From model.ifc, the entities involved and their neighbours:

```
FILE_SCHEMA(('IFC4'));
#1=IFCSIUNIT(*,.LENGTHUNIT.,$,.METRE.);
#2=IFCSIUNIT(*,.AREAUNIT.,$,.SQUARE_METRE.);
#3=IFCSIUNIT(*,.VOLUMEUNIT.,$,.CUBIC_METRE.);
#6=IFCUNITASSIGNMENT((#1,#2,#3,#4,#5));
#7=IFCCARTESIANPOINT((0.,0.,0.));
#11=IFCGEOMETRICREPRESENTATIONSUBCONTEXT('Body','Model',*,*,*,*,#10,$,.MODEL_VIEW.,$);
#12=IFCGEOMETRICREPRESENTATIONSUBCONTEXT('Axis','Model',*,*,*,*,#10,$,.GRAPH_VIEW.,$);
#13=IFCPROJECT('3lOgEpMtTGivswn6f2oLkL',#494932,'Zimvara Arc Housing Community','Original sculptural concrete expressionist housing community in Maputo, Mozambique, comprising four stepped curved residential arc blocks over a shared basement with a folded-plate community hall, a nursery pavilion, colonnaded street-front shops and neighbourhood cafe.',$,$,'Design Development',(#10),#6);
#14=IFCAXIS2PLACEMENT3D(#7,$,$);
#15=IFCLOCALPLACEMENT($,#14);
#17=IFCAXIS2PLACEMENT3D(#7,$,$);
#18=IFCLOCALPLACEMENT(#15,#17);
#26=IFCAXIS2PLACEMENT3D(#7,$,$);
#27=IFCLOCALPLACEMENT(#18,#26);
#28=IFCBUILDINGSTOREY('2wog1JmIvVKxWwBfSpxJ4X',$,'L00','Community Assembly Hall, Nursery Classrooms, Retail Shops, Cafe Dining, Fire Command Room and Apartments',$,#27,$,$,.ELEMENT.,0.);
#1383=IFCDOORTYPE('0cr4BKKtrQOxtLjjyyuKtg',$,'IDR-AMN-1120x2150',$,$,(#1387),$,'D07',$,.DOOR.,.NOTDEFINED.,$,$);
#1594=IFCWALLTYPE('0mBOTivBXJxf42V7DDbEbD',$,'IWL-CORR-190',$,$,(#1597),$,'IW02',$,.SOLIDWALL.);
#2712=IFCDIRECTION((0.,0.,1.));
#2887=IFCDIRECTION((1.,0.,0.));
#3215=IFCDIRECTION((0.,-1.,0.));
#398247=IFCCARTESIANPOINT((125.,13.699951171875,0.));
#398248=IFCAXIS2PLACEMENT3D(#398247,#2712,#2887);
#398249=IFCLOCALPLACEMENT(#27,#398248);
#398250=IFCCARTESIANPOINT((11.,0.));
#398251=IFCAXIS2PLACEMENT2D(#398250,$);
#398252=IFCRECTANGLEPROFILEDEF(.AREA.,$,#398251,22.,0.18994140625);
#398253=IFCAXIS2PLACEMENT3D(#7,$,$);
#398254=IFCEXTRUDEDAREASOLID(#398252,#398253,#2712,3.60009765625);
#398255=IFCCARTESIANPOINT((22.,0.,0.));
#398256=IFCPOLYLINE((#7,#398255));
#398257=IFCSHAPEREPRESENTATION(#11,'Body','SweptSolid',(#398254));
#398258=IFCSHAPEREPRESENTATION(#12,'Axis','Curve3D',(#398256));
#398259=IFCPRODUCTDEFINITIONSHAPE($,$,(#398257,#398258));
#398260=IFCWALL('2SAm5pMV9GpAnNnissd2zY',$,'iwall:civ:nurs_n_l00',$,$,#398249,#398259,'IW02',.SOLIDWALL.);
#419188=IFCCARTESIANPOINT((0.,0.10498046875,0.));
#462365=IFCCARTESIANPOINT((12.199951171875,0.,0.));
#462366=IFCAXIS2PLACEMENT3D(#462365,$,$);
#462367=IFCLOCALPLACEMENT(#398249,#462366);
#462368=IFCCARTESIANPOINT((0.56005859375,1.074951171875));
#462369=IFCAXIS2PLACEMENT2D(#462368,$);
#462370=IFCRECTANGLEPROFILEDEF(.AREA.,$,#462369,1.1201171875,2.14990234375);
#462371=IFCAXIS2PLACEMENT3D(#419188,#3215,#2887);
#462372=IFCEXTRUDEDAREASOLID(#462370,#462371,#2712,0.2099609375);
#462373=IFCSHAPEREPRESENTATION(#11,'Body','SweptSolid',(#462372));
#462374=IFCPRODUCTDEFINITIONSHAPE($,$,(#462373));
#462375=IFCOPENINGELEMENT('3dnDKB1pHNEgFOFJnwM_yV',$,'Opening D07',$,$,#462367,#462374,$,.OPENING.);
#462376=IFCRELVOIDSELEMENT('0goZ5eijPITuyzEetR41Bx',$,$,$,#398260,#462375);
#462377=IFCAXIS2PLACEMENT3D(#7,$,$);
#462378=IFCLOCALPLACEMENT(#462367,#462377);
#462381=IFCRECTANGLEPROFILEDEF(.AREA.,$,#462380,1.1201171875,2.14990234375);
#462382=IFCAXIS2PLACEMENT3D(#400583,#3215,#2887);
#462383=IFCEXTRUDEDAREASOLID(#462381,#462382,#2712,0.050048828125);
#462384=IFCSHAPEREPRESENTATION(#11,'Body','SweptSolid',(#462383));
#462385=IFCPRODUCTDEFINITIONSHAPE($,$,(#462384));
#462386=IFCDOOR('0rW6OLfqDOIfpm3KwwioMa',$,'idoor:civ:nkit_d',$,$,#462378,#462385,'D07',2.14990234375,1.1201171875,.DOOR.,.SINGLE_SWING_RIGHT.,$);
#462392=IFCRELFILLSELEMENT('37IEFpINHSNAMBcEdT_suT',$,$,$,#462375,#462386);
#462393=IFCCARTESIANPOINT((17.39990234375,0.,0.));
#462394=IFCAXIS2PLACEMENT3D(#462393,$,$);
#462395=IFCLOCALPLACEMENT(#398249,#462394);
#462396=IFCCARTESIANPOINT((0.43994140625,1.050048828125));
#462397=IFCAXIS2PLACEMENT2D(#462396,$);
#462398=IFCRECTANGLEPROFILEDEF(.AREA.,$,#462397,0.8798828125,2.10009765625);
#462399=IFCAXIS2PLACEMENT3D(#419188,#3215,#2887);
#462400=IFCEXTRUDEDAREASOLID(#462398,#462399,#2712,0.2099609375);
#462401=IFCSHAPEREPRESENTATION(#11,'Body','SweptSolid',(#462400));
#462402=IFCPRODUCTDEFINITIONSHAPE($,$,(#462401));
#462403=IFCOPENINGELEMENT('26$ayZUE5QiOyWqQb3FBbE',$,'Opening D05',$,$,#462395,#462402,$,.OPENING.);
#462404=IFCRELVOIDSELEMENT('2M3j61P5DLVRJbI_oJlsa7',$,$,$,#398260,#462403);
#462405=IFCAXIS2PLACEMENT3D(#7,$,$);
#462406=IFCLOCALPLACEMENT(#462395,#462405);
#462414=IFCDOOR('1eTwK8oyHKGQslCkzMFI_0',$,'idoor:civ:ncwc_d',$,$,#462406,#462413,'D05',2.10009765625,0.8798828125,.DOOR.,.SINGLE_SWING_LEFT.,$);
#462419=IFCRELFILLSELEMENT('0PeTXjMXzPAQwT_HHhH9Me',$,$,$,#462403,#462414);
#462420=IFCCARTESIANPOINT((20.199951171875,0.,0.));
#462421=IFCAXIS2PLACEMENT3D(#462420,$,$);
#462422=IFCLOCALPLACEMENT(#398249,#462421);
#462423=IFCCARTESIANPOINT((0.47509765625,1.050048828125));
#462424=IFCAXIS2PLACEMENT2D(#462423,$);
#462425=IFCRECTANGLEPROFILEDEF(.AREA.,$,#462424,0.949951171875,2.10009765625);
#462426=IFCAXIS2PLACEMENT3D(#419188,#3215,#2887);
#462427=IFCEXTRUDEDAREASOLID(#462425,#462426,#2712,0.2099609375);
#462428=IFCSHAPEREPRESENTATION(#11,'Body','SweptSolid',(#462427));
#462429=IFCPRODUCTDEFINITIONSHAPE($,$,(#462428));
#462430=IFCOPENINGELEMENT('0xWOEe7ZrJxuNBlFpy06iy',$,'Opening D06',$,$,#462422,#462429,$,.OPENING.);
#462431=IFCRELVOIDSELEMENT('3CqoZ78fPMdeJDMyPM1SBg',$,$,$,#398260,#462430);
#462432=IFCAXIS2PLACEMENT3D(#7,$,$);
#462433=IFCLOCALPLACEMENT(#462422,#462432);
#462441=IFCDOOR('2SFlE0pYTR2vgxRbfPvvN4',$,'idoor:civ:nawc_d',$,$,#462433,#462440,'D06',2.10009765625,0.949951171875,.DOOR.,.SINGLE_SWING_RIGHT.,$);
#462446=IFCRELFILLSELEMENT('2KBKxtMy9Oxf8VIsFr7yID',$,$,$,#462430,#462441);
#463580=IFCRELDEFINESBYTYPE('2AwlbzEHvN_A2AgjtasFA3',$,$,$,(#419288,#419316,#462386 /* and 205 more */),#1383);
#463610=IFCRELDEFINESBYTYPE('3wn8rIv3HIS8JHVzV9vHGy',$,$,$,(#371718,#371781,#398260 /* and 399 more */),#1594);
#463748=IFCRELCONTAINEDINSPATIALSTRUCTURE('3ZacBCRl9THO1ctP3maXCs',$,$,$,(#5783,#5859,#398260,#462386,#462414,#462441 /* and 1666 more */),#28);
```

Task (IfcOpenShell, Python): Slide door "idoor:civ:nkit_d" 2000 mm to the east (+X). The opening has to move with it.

```python
import ifcopenshell
import ifcopenshell.api.geometry
import ifcopenshell.util.placement

model = ifcopenshell.open("model.ifc")

door = model.by_guid("0rW6OLfqDOIfpm3KwwioMa")
opening = door.FillsVoids[0].RelatingOpeningElement
wall = opening.VoidsElements[0].RelatingBuildingElement

wall_matrix = ifcopenshell.util.placement.get_local_placement(wall.ObjectPlacement)
shift = wall_matrix[:3, 0] * 2.0
before = ifcopenshell.util.placement.get_local_placement(door.ObjectPlacement)[:3, 3].copy()

# The door is placed relative to its opening, so it follows when the opening moves.
matrix = ifcopenshell.util.placement.get_local_placement(opening.ObjectPlacement)
matrix[:3, 3] += shift
ifcopenshell.api.geometry.edit_object_placement(
    model, product=opening, matrix=matrix, is_si=False, should_transform_children=True
)

after = ifcopenshell.util.placement.get_local_placement(door.ObjectPlacement)[:3, 3]
print("door moved by", (after - before).round(3) + 0.0)

model.write("model_updated.ifc")
```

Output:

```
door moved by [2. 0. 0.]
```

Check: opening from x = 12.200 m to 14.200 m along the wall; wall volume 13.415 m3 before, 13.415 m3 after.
